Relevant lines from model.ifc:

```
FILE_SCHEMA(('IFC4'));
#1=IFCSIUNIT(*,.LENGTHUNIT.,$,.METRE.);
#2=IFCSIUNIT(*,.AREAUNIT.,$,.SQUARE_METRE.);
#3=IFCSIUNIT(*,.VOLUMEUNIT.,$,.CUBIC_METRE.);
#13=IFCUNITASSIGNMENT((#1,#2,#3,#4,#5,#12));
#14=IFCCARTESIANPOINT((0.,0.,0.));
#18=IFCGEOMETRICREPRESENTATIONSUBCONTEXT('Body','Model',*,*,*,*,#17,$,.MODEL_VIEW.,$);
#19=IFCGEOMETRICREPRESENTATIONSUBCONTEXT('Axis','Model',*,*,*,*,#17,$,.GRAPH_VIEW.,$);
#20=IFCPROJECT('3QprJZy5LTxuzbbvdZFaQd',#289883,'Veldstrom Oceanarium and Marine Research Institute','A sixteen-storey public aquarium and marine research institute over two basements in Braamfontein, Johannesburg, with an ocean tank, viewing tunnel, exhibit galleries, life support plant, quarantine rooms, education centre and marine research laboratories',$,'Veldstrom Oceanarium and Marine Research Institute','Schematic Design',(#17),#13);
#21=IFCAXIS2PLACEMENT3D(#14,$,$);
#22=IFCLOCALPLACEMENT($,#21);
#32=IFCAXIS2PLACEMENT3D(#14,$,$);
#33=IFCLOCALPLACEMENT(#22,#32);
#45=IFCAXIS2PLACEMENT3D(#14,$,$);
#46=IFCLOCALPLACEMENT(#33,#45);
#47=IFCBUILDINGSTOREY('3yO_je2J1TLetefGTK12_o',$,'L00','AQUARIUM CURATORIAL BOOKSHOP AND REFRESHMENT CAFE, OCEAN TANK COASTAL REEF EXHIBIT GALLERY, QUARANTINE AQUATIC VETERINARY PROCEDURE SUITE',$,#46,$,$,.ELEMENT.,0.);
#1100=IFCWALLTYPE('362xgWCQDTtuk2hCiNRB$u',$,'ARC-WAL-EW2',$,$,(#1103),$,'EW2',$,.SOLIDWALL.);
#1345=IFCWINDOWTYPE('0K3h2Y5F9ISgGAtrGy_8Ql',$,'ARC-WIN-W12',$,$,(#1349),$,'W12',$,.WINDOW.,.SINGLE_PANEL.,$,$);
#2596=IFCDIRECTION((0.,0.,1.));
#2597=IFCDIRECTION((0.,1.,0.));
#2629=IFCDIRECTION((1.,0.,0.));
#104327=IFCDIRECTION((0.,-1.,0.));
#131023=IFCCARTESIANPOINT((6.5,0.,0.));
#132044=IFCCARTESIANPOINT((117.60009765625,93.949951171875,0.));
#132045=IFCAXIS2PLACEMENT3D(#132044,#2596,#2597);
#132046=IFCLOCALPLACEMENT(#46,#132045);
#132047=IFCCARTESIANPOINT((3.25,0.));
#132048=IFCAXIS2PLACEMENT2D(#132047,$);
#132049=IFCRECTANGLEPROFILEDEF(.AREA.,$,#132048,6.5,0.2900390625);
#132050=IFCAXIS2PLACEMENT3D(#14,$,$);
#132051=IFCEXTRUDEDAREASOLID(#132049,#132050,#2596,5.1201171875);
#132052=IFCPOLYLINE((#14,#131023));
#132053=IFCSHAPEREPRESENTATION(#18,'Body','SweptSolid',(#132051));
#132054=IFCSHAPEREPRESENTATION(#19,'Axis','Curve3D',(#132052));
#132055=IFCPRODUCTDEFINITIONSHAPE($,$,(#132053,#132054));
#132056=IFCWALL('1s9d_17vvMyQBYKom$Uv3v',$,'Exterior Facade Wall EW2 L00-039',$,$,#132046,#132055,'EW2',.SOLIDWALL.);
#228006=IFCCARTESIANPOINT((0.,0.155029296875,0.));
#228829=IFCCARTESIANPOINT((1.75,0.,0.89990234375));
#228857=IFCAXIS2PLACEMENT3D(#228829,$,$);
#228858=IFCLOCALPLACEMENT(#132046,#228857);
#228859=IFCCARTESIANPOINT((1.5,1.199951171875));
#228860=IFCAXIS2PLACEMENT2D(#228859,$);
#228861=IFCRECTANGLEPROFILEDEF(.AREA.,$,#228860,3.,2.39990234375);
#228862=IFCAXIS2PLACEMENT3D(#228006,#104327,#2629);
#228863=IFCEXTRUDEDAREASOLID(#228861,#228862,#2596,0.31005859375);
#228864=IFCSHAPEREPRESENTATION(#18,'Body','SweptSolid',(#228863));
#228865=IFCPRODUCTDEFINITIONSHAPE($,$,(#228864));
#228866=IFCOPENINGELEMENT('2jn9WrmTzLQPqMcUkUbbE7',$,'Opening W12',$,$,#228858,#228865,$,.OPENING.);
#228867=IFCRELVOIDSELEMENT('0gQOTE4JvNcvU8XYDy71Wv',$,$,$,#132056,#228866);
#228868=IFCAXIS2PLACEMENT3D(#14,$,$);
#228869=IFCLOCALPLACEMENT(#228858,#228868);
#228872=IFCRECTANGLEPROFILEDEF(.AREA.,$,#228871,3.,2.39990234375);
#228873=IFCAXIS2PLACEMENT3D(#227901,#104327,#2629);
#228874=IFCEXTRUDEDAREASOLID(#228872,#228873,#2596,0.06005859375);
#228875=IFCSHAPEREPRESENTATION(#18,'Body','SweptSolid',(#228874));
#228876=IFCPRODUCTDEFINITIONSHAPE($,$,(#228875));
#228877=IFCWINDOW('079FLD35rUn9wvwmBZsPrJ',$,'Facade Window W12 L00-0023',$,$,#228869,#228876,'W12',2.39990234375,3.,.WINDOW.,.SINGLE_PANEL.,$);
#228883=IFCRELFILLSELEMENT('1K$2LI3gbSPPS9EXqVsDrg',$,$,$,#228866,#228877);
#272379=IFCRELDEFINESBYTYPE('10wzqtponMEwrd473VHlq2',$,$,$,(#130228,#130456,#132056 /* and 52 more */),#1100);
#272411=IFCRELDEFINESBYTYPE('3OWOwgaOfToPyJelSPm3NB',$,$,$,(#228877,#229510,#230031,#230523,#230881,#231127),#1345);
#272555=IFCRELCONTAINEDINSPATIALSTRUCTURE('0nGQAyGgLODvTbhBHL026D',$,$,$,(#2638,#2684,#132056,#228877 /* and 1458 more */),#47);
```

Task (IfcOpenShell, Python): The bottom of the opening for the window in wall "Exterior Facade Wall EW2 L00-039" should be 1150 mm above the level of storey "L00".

```python
import numpy as np
import ifcopenshell
import ifcopenshell.api.geometry
import ifcopenshell.geom
import ifcopenshell.util.element
import ifcopenshell.util.placement
import ifcopenshell.util.shape
import ifcopenshell.util.unit

model = ifcopenshell.open("model.ifc")
unit_scale = ifcopenshell.util.unit.calculate_unit_scale(model)

window = model.by_id(228877)
opening = window.FillsVoids[0].RelatingOpeningElement
storey = ifcopenshell.util.element.get_container(window, ifc_class="IfcBuildingStorey")
level = ifcopenshell.util.placement.get_local_placement(storey.ObjectPlacement)[2, 3]

# The opening's origin need not be at the sill, so measure its lowest point.
shape = ifcopenshell.geom.create_shape(ifcopenshell.geom.settings(), opening)
bottom = ifcopenshell.util.shape.get_shape_bottom_elevation(shape, shape.geometry) / unit_scale
dz = level + 1.15 / unit_scale - bottom

shift = np.array([0.0, 0.0, dz])
# The window is placed relative to its opening, so it follows when the opening moves.
matrix = ifcopenshell.util.placement.get_local_placement(opening.ObjectPlacement)
matrix[:3, 3] += shift
ifcopenshell.api.geometry.edit_object_placement(
    model, product=opening, matrix=matrix, is_si=False, should_transform_children=True
)

print(f"moved by {dz * unit_scale:+.3f} m")

model.write("model_v2.ifc")
```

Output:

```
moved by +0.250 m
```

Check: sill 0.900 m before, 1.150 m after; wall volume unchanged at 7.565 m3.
